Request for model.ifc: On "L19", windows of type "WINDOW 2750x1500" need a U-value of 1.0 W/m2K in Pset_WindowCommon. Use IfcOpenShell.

First a look at what the model holds.

```python
import ifcopenshell
import ifcopenshell.util.element

model = ifcopenshell.open("model.ifc")
print(model.schema)
storey = next(s for s in model.by_type("IfcBuildingStorey") if s.Name == "L19")
windows = [e for e in ifcopenshell.util.element.get_decomposition(storey) if e.is_a("IfcWindow")]
seen = {}
for e in windows:
    element_type = ifcopenshell.util.element.get_type(e)
    key = (element_type.Name if element_type != e and element_type else None, ifcopenshell.util.element.get_pset(e, "Pset_WindowCommon", "ThermalTransmittance"))
    seen[key] = seen.get(key, 0) + 1
for (name, value), count in sorted(seen.items(), key=str):
    print(count, "x", name, "|", value)
```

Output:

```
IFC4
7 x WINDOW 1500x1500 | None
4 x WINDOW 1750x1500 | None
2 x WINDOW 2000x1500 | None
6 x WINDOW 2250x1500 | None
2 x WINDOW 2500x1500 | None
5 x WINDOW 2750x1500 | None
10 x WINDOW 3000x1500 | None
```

```python
import ifcopenshell
import ifcopenshell.api.pset
import ifcopenshell.util.element

model = ifcopenshell.open("model.ifc")

storey = next(s for s in model.by_type("IfcBuildingStorey") if s.Name == "L19")
windows = [e for e in ifcopenshell.util.element.get_decomposition(storey) if e.is_a("IfcWindow")]

count = 0
for e in windows:
    element_type = ifcopenshell.util.element.get_type(e)
    if element_type in (None, e) or element_type.Name != "WINDOW 2750x1500":
        continue
    found = ifcopenshell.util.element.get_pset(e, "Pset_WindowCommon", should_inherit=False)
    if found:
        pset = model.by_id(found["id"])
        if len(ifcopenshell.util.element.get_elements_by_pset(pset)) > 1:
            pset = ifcopenshell.api.pset.unshare_pset(model, products=[e], pset=pset)[0]
    else:
        pset = ifcopenshell.api.pset.add_pset(model, product=e, name="Pset_WindowCommon")
    ifcopenshell.api.pset.edit_pset(model, pset=pset, properties={"ThermalTransmittance": 1.0})
    count += 1

print(count, "windows updated")

model.write("model-out.ifc")
```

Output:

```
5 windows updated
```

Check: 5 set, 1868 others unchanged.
